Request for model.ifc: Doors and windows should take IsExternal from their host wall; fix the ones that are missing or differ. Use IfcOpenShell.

First a look at what the model holds.

```python
import ifcopenshell
import ifcopenshell.util.element

model = ifcopenshell.open("model.ifc")
print(model.schema)
seen = {}
for e in model.by_type("IfcDoor") + model.by_type("IfcWindow"):
    if not e.FillsVoids:
        continue
    host = e.FillsVoids[0].RelatingOpeningElement.VoidsElements[0].RelatingBuildingElement
    own = ifcopenshell.util.element.get_pset(e, f"Pset_{e.is_a()[3:].removesuffix('StandardCase')}Common", "IsExternal")
    wall = ifcopenshell.util.element.get_pset(host, "Pset_WallCommon", "IsExternal")
    seen[e.is_a(), own, wall] = seen.get((e.is_a(), own, wall), 0) + 1
for (cls, own, wall), count in sorted(seen.items(), key=str):
    print(count, cls, "IsExternal:", own, "| host wall:", wall)
```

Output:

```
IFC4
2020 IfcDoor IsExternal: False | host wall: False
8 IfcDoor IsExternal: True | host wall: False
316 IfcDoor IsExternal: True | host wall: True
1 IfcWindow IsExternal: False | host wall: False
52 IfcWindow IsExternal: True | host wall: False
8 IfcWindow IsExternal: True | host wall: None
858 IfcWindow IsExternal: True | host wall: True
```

```python
import ifcopenshell
import ifcopenshell.api.pset
import ifcopenshell.util.element

model = ifcopenshell.open("model.ifc")

count = 0
for ifc_class, pset_name in (("IfcDoor", "Pset_DoorCommon"), ("IfcWindow", "Pset_WindowCommon")):
    for e in model.by_type(ifc_class):
        if not e.FillsVoids:
            continue
        host = e.FillsVoids[0].RelatingOpeningElement.VoidsElements[0].RelatingBuildingElement
        external = ifcopenshell.util.element.get_pset(host, "Pset_WallCommon", "IsExternal")
        if external is None or ifcopenshell.util.element.get_pset(e, pset_name, "IsExternal") == external:
            continue
        pset = ifcopenshell.api.pset.add_pset(model, product=e, name=pset_name)
        ifcopenshell.api.pset.edit_pset(model, pset=pset, properties={"IsExternal": external})
        count += 1

print(count, "updated")

model.write("model_updated.ifc")
```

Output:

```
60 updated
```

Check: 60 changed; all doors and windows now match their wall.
